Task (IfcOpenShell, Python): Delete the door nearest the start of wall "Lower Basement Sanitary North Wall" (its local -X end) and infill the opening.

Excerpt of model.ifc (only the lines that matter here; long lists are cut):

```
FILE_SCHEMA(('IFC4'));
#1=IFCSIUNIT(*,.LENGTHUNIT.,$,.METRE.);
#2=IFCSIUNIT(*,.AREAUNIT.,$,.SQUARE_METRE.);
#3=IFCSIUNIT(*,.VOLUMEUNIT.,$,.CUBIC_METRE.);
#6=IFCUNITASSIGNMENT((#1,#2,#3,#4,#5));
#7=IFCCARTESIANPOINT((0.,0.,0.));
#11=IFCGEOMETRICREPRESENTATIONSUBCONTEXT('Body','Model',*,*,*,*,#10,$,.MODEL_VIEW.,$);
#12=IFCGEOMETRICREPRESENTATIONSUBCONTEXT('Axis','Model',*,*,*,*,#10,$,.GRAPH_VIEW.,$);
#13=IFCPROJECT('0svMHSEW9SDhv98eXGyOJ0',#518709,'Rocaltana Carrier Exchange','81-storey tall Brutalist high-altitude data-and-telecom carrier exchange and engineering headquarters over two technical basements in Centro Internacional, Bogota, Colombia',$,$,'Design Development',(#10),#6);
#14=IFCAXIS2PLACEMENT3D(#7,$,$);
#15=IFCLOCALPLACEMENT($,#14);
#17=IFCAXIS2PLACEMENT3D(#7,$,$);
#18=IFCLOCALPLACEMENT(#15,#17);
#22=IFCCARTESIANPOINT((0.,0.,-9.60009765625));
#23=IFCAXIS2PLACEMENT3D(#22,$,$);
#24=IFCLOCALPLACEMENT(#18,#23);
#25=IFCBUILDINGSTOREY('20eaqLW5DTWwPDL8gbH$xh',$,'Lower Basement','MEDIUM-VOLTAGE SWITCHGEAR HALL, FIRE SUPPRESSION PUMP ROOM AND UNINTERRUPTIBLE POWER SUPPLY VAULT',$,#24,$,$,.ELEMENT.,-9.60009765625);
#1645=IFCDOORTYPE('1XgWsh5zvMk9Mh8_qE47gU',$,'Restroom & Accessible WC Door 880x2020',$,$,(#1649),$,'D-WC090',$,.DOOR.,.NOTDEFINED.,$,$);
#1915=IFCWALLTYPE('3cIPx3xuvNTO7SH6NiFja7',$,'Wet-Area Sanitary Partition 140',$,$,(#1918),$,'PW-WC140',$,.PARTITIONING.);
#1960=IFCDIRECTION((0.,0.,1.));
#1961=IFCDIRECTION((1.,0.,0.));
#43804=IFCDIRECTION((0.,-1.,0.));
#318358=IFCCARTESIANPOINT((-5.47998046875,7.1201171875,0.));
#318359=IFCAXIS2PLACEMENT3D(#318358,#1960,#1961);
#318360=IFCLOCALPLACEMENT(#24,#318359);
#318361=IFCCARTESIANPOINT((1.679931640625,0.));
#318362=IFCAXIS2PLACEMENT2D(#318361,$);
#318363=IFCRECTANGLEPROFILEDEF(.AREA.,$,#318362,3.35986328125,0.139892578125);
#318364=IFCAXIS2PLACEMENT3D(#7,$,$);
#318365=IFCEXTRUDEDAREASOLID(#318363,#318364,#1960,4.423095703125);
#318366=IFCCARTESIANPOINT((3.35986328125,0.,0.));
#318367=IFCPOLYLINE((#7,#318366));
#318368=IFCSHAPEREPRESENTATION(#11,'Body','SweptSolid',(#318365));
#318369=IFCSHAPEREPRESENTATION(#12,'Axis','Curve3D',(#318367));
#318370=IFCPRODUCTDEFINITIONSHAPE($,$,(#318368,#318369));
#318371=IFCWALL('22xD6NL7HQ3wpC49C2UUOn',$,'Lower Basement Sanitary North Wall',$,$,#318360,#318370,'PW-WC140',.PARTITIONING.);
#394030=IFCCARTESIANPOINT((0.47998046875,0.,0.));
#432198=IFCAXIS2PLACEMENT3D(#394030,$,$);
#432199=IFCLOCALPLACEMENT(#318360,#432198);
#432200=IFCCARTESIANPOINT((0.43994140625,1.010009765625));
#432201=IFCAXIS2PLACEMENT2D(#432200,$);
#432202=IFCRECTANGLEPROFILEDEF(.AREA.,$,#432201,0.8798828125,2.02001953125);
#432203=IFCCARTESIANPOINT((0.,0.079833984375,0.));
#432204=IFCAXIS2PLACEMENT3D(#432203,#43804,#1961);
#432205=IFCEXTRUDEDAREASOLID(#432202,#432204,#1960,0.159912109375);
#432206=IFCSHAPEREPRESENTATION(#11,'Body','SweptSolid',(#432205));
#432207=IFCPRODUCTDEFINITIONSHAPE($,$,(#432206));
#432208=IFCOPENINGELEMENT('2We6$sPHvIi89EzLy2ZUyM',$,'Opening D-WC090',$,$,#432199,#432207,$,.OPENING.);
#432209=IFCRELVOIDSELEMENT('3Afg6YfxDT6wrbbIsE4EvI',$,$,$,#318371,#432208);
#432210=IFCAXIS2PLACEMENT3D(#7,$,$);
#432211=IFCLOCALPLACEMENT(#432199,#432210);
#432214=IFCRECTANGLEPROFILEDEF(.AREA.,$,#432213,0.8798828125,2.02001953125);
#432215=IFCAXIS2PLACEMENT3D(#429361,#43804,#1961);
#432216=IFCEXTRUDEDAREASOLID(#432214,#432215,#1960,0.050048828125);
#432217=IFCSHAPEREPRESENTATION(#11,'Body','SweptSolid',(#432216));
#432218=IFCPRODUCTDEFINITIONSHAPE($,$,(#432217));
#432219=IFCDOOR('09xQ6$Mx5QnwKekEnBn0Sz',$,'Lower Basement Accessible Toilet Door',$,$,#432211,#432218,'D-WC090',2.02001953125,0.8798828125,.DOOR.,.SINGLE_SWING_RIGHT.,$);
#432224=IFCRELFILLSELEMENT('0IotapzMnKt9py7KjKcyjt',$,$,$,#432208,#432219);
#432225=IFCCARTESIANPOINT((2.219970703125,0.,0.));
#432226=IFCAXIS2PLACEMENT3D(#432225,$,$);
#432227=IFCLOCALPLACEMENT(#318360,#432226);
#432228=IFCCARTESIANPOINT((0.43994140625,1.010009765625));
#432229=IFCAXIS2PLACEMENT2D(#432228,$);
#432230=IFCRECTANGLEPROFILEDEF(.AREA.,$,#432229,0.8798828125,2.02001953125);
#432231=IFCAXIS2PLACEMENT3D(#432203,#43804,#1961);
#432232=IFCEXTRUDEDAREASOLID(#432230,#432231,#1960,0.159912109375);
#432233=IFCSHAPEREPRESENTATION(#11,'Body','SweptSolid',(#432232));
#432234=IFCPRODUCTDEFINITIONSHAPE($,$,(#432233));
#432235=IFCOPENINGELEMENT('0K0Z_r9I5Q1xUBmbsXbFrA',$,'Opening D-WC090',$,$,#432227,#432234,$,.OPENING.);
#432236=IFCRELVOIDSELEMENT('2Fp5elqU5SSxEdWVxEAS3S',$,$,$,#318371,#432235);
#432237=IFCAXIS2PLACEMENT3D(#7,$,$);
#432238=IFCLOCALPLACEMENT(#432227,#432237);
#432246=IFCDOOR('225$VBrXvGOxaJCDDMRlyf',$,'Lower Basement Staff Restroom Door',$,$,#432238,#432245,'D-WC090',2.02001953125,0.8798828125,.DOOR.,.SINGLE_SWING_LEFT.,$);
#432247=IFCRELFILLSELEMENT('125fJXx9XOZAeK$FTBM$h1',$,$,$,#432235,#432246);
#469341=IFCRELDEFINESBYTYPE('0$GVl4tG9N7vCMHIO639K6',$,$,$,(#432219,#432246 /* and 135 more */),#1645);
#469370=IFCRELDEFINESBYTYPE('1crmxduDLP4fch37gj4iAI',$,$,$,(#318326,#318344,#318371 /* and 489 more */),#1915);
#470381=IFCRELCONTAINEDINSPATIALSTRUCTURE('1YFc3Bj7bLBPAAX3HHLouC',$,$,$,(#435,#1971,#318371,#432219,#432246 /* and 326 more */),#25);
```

```python
import ifcopenshell
import ifcopenshell.api.feature
import ifcopenshell.api.root
import ifcopenshell.geom
import ifcopenshell.util.shape

model = ifcopenshell.open("model.ifc")
settings = ifcopenshell.geom.settings()


def volume(element):
    """Net volume in cubic metres, openings subtracted."""
    shape = ifcopenshell.geom.create_shape(settings, element)
    return ifcopenshell.util.shape.get_volume(shape.geometry)


door = model.by_guid("09xQ6$Mx5QnwKekEnBn0Sz")
opening = door.FillsVoids[0].RelatingOpeningElement
wall = opening.VoidsElements[0].RelatingBuildingElement
before = volume(wall)

ifcopenshell.api.root.remove_product(model, product=door)
ifcopenshell.api.feature.remove_feature(model, feature=opening)

after = volume(wall)

print(f"wall volume {before:.3f} -> {after:.3f} m3")

model.write("model_rev.ifc")
```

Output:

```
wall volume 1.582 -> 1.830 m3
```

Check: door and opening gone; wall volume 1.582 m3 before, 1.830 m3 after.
